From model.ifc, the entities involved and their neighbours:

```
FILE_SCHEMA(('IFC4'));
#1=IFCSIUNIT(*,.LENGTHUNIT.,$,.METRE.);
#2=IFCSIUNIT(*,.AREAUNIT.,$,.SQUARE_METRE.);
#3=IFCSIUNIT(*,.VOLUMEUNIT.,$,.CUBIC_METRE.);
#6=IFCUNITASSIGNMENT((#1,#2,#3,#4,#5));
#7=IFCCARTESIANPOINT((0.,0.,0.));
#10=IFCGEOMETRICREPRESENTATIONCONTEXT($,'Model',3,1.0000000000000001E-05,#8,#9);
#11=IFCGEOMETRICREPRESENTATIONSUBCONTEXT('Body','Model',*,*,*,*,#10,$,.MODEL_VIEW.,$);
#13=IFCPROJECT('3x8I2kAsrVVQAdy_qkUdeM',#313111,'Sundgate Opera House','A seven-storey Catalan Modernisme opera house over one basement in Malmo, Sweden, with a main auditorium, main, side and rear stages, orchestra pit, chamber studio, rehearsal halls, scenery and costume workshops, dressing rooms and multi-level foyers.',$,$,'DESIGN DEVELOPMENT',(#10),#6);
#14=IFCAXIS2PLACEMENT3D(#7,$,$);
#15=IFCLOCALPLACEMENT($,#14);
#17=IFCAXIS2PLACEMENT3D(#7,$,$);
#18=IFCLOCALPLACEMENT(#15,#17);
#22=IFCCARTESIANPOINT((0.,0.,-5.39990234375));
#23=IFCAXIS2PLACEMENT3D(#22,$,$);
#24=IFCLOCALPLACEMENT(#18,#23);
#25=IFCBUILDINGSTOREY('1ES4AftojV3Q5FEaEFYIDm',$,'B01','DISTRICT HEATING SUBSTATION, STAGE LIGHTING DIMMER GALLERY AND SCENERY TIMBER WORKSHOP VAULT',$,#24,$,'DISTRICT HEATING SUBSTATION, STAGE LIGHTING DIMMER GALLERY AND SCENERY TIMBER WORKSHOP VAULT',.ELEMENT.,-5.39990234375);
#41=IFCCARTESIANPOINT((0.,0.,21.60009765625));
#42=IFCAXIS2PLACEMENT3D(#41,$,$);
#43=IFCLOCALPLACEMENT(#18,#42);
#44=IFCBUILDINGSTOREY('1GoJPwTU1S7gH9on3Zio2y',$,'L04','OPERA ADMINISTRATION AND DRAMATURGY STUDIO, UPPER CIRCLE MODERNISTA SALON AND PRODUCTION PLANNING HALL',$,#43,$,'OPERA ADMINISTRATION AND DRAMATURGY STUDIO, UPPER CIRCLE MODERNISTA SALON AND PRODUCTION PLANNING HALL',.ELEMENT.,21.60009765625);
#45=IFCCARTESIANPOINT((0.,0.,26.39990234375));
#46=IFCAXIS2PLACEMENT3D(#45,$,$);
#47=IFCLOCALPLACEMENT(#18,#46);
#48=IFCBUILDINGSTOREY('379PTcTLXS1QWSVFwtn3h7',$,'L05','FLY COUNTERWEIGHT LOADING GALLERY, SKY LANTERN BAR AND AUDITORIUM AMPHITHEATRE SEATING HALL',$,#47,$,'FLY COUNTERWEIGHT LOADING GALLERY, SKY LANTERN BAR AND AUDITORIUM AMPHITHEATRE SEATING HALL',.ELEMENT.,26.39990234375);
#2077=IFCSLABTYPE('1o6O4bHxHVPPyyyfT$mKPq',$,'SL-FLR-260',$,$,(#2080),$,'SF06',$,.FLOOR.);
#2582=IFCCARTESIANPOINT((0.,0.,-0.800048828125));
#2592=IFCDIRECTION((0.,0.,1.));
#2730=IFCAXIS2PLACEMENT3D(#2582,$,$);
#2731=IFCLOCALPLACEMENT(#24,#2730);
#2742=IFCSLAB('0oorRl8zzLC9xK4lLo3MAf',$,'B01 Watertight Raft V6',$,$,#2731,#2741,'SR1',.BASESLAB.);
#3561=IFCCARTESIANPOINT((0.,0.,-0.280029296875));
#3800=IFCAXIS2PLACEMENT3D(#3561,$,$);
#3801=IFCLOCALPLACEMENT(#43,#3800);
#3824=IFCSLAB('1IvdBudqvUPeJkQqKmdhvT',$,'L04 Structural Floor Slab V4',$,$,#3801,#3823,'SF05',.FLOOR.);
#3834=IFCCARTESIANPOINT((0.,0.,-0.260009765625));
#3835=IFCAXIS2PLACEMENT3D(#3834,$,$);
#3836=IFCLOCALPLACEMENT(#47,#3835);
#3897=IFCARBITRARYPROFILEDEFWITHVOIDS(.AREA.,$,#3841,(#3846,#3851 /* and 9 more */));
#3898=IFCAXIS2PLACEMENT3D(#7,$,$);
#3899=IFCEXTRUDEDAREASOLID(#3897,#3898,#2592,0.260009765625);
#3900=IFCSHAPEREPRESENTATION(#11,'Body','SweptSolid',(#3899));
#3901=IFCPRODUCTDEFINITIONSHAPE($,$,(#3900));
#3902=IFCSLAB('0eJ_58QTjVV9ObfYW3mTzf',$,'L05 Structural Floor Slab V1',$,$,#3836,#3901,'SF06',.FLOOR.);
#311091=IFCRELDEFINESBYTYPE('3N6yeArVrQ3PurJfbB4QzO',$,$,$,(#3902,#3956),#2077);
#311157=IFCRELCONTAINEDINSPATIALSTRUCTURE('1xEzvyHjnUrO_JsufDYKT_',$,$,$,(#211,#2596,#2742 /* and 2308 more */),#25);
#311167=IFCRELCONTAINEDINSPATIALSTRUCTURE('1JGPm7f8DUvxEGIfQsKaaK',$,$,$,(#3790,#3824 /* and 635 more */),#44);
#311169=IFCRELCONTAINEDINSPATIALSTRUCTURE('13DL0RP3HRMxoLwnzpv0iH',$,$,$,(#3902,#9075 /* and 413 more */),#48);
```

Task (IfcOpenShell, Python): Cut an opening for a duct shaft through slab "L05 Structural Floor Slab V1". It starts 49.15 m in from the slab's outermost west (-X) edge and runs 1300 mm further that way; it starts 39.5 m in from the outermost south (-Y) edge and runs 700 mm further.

```python
import numpy as np
import ifcopenshell
import ifcopenshell.api.feature
import ifcopenshell.api.geometry
import ifcopenshell.api.root
import ifcopenshell.geom
import ifcopenshell.util.placement
import ifcopenshell.util.representation
import ifcopenshell.util.shape
import ifcopenshell.util.unit

model = ifcopenshell.open("model.ifc")
unit_scale = ifcopenshell.util.unit.calculate_unit_scale(model)
settings = ifcopenshell.geom.settings()


def volume(element):
    """Net volume in cubic metres, openings subtracted."""
    shape = ifcopenshell.geom.create_shape(settings, element)
    return ifcopenshell.util.shape.get_volume(shape.geometry)


slab = model.by_id(3902)
before = volume(slab)

# Extent in the slab's own axes, in metres. The edges named are its -X and -Y sides.
slab_shape = ifcopenshell.geom.create_shape(settings, slab)
vertices = ifcopenshell.util.shape.get_vertices(slab_shape.geometry)
x_min, y_min, bottom = vertices.min(axis=0)
top = vertices[:, 2].max()

opening = ifcopenshell.api.root.create_entity(model, ifc_class="IfcOpeningElement", name="Duct shaft opening", predefined_type="OPENING")
context = ifcopenshell.util.representation.get_context(model, "Model", "Body", "MODEL_VIEW")
width, depth = 1.3, 0.7
outline = [(0.0, 0.0), (width, 0.0), (width, depth), (0.0, depth), (0.0, 0.0)]
# Overshoot both faces by 50 mm so the cut is clean.
shape = ifcopenshell.api.geometry.add_slab_representation(
    model, context=context, depth=top - bottom + 0.1, polyline=outline
)
ifcopenshell.api.geometry.assign_representation(model, product=opening, representation=shape)

matrix = ifcopenshell.util.placement.get_local_placement(slab.ObjectPlacement)
matrix[:, 3] = matrix @ np.append(np.array([x_min + 49.15, y_min + 39.5, bottom - 0.05]) / unit_scale, 1.0)
ifcopenshell.api.geometry.edit_object_placement(model, product=opening, matrix=matrix, is_si=False)
ifcopenshell.api.feature.add_feature(model, feature=opening, element=slab)

after = volume(slab)

print(f"slab volume {before:.3f} -> {after:.3f} m3")

model.write("model_v2.ifc")
```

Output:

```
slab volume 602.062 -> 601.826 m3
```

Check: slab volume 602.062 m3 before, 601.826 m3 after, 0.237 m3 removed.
